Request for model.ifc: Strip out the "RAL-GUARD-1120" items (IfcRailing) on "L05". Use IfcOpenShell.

First a look at what the model holds.

```python
import ifcopenshell
import ifcopenshell.util.element

model = ifcopenshell.open("model.ifc")
print(model.schema)
storey = next(s for s in model.by_type("IfcBuildingStorey") if s.Name == "L05")
railings = [e for e in ifcopenshell.util.element.get_decomposition(storey) if e.is_a("IfcRailing")]
seen = {}
for e in railings:
    element_type = ifcopenshell.util.element.get_type(e)
    name = element_type.Name if element_type not in (None, e) else None
    seen[name] = seen.get(name, 0) + 1
for name, count in sorted(seen.items(), key=str):
    print(count, "x", name)
```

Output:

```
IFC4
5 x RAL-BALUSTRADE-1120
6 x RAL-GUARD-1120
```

```python
import ifcopenshell
import ifcopenshell.api.root
import ifcopenshell.util.element

model = ifcopenshell.open("model.ifc")

storey = next(s for s in model.by_type("IfcBuildingStorey") if s.Name == "L05")
railings = [e for e in ifcopenshell.util.element.get_decomposition(storey) if e.is_a("IfcRailing")]
targets = [e for e in railings if (t := ifcopenshell.util.element.get_type(e)) not in (None, e) and t.Name == "RAL-GUARD-1120"]

for e in targets:
    ifcopenshell.api.root.remove_product(model, product=e)
print(len(targets), "removed")

model.write("model-out.ifc")
```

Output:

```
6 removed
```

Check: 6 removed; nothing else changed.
